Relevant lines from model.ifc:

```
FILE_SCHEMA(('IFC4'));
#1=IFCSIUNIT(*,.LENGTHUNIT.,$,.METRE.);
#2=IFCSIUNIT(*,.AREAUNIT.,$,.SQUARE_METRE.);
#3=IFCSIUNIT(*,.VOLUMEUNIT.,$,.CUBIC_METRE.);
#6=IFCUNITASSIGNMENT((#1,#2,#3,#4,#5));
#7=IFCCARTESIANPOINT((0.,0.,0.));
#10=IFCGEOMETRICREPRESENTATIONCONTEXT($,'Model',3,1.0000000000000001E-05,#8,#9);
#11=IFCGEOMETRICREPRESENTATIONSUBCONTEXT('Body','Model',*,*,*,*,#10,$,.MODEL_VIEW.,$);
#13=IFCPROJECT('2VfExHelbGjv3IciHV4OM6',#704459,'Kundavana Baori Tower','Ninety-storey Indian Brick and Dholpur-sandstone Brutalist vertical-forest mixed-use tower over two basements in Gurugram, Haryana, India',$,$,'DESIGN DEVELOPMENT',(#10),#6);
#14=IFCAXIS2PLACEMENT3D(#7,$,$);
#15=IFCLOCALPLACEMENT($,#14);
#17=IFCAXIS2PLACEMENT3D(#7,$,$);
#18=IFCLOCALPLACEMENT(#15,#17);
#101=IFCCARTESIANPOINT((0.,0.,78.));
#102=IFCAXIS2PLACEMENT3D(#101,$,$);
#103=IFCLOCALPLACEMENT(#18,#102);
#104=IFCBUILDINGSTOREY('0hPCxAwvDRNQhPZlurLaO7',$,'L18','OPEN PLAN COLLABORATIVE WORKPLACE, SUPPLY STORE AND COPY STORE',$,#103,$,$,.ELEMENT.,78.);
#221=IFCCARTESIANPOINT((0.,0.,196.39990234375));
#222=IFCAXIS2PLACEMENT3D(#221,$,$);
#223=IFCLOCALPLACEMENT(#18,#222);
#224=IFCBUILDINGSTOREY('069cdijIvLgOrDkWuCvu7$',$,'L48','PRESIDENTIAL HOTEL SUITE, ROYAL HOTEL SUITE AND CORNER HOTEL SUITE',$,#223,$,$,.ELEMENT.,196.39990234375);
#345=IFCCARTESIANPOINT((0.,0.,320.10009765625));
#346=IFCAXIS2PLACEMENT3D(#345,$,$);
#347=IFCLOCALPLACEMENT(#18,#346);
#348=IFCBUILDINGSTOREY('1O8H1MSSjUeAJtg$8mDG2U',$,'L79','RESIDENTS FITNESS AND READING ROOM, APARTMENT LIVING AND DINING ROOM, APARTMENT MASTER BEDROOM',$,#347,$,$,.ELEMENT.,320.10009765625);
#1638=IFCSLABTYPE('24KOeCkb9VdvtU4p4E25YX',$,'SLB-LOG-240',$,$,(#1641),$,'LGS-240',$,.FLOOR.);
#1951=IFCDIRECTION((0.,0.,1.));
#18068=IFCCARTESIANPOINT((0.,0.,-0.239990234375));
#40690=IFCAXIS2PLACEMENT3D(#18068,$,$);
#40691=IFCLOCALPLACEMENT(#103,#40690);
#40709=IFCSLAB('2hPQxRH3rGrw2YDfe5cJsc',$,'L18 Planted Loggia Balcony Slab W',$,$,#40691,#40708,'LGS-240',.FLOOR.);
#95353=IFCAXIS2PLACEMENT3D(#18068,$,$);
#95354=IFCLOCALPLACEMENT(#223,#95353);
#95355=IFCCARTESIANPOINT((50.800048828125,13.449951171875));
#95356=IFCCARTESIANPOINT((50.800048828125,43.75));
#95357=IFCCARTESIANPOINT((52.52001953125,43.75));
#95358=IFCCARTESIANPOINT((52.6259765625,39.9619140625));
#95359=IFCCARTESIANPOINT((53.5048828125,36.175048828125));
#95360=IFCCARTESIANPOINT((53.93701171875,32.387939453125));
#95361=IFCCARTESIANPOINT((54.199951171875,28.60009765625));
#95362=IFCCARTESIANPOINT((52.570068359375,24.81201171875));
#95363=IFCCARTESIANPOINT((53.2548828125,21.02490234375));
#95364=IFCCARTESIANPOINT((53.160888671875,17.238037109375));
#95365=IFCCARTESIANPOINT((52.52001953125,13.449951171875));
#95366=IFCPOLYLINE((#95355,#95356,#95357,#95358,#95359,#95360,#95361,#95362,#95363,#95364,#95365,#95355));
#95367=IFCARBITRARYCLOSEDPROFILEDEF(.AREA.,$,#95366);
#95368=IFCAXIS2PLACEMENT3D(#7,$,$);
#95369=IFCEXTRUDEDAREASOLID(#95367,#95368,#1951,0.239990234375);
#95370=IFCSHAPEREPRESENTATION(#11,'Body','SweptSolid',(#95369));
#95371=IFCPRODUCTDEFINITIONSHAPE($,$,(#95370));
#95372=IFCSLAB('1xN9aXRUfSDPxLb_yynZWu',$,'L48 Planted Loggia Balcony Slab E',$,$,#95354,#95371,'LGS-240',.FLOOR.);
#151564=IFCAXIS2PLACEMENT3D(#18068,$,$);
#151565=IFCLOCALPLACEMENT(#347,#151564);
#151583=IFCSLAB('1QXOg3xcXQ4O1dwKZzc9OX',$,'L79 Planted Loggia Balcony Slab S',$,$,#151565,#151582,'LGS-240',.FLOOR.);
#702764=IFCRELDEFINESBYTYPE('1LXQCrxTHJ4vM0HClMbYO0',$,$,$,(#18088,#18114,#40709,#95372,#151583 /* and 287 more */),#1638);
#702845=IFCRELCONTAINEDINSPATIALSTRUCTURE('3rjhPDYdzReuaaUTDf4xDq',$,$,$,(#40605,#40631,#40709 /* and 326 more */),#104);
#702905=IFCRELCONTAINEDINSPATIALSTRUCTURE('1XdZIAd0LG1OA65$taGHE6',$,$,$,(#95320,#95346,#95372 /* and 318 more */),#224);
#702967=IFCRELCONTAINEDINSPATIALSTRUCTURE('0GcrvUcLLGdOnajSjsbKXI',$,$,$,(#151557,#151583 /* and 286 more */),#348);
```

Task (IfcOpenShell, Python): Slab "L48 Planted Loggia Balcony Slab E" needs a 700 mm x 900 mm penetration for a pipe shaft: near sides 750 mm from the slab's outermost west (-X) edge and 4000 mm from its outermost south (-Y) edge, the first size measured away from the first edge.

```python
import numpy as np
import ifcopenshell
import ifcopenshell.api.feature
import ifcopenshell.api.geometry
import ifcopenshell.api.root
import ifcopenshell.geom
import ifcopenshell.util.placement
import ifcopenshell.util.representation
import ifcopenshell.util.shape
import ifcopenshell.util.unit

model = ifcopenshell.open("model.ifc")
unit_scale = ifcopenshell.util.unit.calculate_unit_scale(model)
settings = ifcopenshell.geom.settings()


def volume(element):
    """Net volume in cubic metres, openings subtracted."""
    shape = ifcopenshell.geom.create_shape(settings, element)
    return ifcopenshell.util.shape.get_volume(shape.geometry)


slab = model.by_id(95372)
before = volume(slab)

# Extent in the slab's own axes, in metres. The edges named are its -X and -Y sides.
slab_shape = ifcopenshell.geom.create_shape(settings, slab)
vertices = ifcopenshell.util.shape.get_vertices(slab_shape.geometry)
x_min, y_min, bottom = vertices.min(axis=0)
top = vertices[:, 2].max()

opening = ifcopenshell.api.root.create_entity(model, ifc_class="IfcOpeningElement", name="Pipe shaft opening", predefined_type="OPENING")
context = ifcopenshell.util.representation.get_context(model, "Model", "Body", "MODEL_VIEW")
width, depth = 0.7, 0.9
outline = [(0.0, 0.0), (width, 0.0), (width, depth), (0.0, depth), (0.0, 0.0)]
# Overshoot both faces by 50 mm so the cut is clean.
shape = ifcopenshell.api.geometry.add_slab_representation(
    model, context=context, depth=top - bottom + 0.1, polyline=outline
)
ifcopenshell.api.geometry.assign_representation(model, product=opening, representation=shape)

matrix = ifcopenshell.util.placement.get_local_placement(slab.ObjectPlacement)
matrix[:, 3] = matrix @ np.append(np.array([x_min + 0.75, y_min + 4, bottom - 0.05]) / unit_scale, 1.0)
ifcopenshell.api.geometry.edit_object_placement(model, product=opening, matrix=matrix, is_si=False)
ifcopenshell.api.feature.add_feature(model, feature=opening, element=slab)

after = volume(slab)

print(f"slab volume {before:.3f} -> {after:.3f} m3")

model.write("model_updated.ifc")
```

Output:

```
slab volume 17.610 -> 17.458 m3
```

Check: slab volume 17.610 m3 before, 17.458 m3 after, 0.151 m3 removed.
